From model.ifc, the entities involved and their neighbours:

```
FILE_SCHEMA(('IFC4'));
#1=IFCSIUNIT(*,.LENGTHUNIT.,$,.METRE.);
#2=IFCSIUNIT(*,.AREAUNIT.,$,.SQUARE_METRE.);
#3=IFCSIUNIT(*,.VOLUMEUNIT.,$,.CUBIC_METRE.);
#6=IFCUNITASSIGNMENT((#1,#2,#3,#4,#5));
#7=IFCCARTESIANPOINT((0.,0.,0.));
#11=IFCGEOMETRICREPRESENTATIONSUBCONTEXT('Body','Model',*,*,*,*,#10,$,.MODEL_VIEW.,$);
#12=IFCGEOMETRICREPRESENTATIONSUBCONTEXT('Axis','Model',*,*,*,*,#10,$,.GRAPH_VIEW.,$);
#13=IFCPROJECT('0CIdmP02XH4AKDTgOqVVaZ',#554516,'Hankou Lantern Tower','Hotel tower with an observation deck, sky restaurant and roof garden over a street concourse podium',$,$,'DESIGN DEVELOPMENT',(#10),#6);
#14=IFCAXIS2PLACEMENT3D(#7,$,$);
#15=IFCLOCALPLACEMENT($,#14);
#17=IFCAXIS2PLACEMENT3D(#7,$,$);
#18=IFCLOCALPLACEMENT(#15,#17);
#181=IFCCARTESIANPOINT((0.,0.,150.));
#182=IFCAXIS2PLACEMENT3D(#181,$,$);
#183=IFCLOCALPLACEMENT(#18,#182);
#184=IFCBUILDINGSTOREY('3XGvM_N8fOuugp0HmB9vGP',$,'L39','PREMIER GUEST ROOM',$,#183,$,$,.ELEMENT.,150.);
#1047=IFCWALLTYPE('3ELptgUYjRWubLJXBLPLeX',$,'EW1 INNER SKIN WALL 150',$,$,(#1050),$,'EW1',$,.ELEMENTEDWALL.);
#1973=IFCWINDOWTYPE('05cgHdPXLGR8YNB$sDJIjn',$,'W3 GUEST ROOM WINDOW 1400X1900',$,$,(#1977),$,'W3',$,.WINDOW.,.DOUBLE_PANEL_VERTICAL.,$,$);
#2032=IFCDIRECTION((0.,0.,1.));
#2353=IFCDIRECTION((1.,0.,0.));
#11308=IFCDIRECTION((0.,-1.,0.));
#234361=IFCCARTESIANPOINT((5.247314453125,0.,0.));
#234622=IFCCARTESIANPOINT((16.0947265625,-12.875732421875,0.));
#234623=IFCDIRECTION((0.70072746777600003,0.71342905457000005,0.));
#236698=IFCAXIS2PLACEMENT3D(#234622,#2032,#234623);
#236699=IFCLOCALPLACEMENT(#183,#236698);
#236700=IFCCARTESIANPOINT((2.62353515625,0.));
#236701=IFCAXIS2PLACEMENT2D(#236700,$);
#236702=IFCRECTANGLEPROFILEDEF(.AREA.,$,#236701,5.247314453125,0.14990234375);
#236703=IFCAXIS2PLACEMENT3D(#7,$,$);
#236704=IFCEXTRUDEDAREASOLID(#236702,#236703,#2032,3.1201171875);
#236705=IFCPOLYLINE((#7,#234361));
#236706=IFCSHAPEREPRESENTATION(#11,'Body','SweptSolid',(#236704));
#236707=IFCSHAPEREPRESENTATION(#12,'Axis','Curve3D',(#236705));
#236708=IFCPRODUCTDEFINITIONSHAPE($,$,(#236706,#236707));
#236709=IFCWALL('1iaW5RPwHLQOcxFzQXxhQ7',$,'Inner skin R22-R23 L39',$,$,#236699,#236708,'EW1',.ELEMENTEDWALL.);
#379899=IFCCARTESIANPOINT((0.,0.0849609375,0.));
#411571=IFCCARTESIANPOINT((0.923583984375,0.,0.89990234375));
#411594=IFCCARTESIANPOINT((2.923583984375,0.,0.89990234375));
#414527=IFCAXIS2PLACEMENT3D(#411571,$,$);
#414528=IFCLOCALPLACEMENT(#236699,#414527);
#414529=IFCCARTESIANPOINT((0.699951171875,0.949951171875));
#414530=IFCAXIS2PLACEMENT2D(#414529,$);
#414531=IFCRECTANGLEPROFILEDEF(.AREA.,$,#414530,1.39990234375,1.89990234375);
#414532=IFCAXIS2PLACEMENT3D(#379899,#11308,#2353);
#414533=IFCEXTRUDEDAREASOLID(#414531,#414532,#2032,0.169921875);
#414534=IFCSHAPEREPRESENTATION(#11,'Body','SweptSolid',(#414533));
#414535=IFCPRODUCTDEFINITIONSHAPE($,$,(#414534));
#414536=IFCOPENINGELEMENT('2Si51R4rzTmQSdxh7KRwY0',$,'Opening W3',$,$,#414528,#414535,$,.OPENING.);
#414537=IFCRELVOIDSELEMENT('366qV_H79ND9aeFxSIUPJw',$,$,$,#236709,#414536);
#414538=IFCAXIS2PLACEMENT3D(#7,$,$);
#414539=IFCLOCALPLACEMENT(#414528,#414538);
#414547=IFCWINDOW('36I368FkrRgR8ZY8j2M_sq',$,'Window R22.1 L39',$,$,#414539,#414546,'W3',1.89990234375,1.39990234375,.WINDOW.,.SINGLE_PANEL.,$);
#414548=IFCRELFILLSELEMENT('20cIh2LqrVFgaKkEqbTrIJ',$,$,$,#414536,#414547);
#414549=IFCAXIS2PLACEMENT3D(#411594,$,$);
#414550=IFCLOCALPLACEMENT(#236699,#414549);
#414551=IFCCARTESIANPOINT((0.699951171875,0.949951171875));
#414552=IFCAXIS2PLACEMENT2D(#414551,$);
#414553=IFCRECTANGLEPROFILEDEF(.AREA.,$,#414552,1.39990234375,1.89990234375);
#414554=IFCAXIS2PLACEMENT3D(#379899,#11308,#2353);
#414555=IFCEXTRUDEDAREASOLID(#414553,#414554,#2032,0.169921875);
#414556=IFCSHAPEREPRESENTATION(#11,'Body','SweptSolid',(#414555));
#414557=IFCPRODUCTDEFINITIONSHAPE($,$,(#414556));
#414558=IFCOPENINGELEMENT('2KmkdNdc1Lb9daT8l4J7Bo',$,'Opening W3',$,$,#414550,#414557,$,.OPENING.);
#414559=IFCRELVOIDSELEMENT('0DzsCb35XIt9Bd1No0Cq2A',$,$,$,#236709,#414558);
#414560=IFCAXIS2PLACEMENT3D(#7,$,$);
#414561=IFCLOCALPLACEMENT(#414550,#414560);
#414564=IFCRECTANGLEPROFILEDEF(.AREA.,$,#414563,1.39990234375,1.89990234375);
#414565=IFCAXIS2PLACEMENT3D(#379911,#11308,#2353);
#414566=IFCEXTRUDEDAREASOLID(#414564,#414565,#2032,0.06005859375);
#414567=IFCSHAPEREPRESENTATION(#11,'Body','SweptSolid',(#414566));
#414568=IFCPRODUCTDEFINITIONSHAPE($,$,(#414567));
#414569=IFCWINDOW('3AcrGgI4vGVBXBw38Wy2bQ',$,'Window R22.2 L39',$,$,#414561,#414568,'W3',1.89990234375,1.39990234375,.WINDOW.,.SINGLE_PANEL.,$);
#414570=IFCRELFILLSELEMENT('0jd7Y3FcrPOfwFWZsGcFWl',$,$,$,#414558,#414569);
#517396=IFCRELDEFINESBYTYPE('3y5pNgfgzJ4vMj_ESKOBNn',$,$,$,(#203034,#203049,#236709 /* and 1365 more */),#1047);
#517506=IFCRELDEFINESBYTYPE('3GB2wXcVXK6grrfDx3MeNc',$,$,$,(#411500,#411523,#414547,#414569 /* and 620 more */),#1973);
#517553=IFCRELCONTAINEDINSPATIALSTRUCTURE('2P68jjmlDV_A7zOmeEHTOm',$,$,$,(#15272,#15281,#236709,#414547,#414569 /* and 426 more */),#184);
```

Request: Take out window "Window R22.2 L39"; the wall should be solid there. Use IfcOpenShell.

```python
import ifcopenshell
import ifcopenshell.api.feature
import ifcopenshell.api.root
import ifcopenshell.geom
import ifcopenshell.util.shape

model = ifcopenshell.open("model.ifc")
settings = ifcopenshell.geom.settings()


def volume(element):
    """Net volume in cubic metres, openings subtracted."""
    shape = ifcopenshell.geom.create_shape(settings, element)
    return ifcopenshell.util.shape.get_volume(shape.geometry)


window = model.by_guid("3AcrGgI4vGVBXBw38Wy2bQ")
opening = window.FillsVoids[0].RelatingOpeningElement
wall = opening.VoidsElements[0].RelatingBuildingElement
before = volume(wall)

ifcopenshell.api.root.remove_product(model, product=window)
ifcopenshell.api.feature.remove_feature(model, feature=opening)

after = volume(wall)

print(f"wall volume {before:.3f} -> {after:.3f} m3")

model.write("model_edited.ifc")
```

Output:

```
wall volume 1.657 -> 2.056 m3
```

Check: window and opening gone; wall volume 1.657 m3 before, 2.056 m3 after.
